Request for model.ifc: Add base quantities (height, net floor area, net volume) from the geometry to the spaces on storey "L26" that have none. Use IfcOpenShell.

First a look at what the model holds.

```python
import ifcopenshell
import ifcopenshell.util.element
import ifcopenshell.util.unit

model = ifcopenshell.open("model.ifc")
print(model.schema)
for unit_type in ("LENGTHUNIT", "AREAUNIT", "VOLUMEUNIT"):
    print(unit_type, ifcopenshell.util.unit.calculate_unit_scale(model, unit_type))
storey = next(s for s in model.by_type("IfcBuildingStorey") if s.Name == "L26")
spaces = [e for e in ifcopenshell.util.element.get_decomposition(storey) if e.is_a("IfcSpace")]
for e in sorted(spaces, key=lambda e: e.id()):
    print(e.id(), e.is_a(), e.Name, list(ifcopenshell.util.element.get_psets(e, qtos_only=True)), sep=" | ")
```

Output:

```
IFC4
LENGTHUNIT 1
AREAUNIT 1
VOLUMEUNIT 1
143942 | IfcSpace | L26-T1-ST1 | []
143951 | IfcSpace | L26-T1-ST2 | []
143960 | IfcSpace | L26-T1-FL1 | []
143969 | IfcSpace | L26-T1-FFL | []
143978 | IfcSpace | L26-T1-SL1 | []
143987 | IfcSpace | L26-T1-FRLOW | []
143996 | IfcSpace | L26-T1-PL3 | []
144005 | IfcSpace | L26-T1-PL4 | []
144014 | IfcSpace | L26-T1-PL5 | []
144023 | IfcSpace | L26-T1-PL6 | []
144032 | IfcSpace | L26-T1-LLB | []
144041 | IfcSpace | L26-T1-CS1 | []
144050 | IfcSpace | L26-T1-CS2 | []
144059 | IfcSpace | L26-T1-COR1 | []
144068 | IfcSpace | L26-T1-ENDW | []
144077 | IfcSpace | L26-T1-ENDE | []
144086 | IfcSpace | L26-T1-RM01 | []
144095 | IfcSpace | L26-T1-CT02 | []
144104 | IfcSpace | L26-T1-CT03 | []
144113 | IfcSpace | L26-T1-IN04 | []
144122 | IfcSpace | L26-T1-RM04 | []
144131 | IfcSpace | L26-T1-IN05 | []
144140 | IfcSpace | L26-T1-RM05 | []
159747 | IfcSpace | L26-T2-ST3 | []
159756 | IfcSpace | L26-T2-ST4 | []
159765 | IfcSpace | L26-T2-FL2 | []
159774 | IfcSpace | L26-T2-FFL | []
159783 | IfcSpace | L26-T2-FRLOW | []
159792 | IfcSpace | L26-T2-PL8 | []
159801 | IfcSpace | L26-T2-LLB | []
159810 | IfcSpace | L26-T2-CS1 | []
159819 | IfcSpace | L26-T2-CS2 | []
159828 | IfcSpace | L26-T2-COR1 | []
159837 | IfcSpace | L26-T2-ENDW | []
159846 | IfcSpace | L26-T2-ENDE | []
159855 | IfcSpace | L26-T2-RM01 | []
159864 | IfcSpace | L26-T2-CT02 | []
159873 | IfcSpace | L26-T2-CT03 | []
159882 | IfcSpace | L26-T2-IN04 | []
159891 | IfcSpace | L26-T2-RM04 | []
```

```python
import ifcopenshell
import ifcopenshell.api.pset
import ifcopenshell.geom
import ifcopenshell.util.element
import ifcopenshell.util.shape
import ifcopenshell.util.unit

model = ifcopenshell.open("model.ifc")
unit_scale = ifcopenshell.util.unit.calculate_unit_scale(model)
area_scale = ifcopenshell.util.unit.calculate_unit_scale(model, "AREAUNIT")
volume_scale = ifcopenshell.util.unit.calculate_unit_scale(model, "VOLUMEUNIT")
settings = ifcopenshell.geom.settings()

storey = next(s for s in model.by_type("IfcBuildingStorey") if s.Name == "L26")
spaces = [e for e in ifcopenshell.util.element.get_decomposition(storey) if e.is_a("IfcSpace")]

for e in sorted(spaces, key=lambda e: e.id()):
    if ifcopenshell.util.element.get_psets(e, qtos_only=True, should_inherit=False):
        continue
    # Geometry comes back in metres, in the element's own axes.
    shape = ifcopenshell.geom.create_shape(settings, e)
    values = {
        "Height": ifcopenshell.util.shape.get_z(shape.geometry) / unit_scale,
        "NetFloorArea": ifcopenshell.util.shape.get_footprint_area(shape.geometry) / area_scale,
        "NetVolume": ifcopenshell.util.shape.get_volume(shape.geometry) / volume_scale,
    }
    qto = ifcopenshell.api.pset.add_qto(model, product=e, name="Qto_SpaceBaseQuantities")
    ifcopenshell.api.pset.edit_qto(model, qto=qto, properties=values)
    print(e.id(), {k: round(v, 3) for k, v in values.items()})

model.write("model_rev.ifc")
```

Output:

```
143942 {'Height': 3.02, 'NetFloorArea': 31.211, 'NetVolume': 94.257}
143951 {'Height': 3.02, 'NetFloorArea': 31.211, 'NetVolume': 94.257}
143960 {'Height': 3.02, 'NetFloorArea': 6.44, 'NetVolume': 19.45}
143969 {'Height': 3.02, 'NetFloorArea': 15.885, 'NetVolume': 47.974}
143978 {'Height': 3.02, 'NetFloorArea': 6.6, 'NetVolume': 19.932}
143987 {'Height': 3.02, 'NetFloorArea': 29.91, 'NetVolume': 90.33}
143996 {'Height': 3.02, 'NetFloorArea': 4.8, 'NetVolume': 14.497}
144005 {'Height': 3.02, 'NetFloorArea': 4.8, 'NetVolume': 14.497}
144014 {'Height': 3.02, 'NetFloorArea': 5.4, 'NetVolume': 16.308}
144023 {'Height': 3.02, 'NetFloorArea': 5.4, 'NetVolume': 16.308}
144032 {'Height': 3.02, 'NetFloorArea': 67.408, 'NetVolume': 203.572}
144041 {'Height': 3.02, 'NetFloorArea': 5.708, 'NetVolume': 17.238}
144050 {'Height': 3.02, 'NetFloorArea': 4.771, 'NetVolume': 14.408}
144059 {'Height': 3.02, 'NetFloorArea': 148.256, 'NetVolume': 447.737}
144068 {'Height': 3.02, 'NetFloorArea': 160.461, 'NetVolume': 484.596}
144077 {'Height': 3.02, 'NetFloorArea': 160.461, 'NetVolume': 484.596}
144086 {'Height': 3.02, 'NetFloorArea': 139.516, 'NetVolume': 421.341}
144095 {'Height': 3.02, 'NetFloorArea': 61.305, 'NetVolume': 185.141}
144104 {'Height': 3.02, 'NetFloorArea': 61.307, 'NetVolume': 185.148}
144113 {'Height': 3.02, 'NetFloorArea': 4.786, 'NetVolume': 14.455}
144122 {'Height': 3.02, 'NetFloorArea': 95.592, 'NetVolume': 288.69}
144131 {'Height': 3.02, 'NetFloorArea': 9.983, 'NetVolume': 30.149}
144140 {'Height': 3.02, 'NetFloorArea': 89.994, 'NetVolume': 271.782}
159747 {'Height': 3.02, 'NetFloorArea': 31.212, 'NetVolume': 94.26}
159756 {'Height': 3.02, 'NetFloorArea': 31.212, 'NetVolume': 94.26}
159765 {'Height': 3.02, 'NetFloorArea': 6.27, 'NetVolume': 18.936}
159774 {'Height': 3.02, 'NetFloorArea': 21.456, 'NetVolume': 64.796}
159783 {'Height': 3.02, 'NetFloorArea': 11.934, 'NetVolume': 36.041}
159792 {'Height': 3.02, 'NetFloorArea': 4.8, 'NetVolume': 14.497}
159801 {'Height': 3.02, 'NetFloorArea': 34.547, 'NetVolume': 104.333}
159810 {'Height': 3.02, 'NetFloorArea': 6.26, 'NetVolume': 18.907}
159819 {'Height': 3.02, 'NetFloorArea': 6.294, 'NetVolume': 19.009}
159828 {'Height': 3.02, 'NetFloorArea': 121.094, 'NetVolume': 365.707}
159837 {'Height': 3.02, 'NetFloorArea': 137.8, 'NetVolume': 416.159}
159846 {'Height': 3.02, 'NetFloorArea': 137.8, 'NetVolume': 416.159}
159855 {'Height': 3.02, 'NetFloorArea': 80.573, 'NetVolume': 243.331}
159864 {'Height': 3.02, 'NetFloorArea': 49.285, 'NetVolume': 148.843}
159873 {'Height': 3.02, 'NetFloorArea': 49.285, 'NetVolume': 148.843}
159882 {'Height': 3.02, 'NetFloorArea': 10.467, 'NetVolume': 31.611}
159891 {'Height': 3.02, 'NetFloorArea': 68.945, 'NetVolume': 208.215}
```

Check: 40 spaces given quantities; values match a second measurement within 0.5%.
